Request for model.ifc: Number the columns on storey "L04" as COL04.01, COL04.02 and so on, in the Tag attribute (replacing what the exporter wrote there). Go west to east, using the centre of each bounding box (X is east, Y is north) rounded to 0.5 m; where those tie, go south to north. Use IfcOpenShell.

First a look at what the model holds.

```python
import ifcopenshell
import ifcopenshell.util.element
import ifcopenshell.util.placement

model = ifcopenshell.open("model.ifc")
print(model.schema)
storey = next(s for s in model.by_type("IfcBuildingStorey") if s.Name == "L04")
columns = [e for e in ifcopenshell.util.element.get_decomposition(storey) if e.is_a("IfcColumn")]
for e in sorted(columns, key=lambda e: e.id()):
    origin = ifcopenshell.util.placement.get_local_placement(e.ObjectPlacement)[:3, 3]
    print(e.id(), e.Tag, e.Name, origin.round(2) + 0.0, sep=" | ")
```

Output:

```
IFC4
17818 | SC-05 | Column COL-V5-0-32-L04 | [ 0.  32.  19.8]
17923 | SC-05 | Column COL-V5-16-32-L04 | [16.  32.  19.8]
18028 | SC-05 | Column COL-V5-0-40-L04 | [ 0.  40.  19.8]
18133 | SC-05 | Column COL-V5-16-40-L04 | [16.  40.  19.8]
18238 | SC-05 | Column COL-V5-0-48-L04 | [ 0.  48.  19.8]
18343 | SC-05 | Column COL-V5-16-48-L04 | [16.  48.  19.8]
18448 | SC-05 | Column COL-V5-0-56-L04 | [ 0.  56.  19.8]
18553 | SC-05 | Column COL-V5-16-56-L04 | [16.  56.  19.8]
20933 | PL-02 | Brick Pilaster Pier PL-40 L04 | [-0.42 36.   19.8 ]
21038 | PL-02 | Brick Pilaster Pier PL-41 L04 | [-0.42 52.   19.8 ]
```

```python
import ifcopenshell
import ifcopenshell.geom
import ifcopenshell.util.element
import ifcopenshell.util.shape

model = ifcopenshell.open("model.ifc")
settings = ifcopenshell.geom.settings()
settings.set("use-world-coords", True)


def centre(element):
    shape = ifcopenshell.geom.create_shape(settings, element)
    return ifcopenshell.util.shape.get_bbox_centroid(shape.geometry)


storey = next(s for s in model.by_type("IfcBuildingStorey") if s.Name == "L04")
columns = [e for e in ifcopenshell.util.element.get_decomposition(storey) if e.is_a("IfcColumn")]

# Insertion points can sit at a corner or the storey origin, so sort by the geometry (in metres).
centres = {e: centre(e) for e in columns}
columns.sort(key=lambda e: (round(centres[e][0] / 0.5), centres[e][1]))

for i, e in enumerate(columns, start=1):
    number = f"COL04.{i:02d}"
    e.Tag = number
    print(e.id(), number)

model.write("model_v2.ifc")
```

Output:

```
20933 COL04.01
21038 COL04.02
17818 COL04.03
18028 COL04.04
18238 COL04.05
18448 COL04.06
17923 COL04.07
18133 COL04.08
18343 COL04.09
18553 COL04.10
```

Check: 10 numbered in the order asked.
